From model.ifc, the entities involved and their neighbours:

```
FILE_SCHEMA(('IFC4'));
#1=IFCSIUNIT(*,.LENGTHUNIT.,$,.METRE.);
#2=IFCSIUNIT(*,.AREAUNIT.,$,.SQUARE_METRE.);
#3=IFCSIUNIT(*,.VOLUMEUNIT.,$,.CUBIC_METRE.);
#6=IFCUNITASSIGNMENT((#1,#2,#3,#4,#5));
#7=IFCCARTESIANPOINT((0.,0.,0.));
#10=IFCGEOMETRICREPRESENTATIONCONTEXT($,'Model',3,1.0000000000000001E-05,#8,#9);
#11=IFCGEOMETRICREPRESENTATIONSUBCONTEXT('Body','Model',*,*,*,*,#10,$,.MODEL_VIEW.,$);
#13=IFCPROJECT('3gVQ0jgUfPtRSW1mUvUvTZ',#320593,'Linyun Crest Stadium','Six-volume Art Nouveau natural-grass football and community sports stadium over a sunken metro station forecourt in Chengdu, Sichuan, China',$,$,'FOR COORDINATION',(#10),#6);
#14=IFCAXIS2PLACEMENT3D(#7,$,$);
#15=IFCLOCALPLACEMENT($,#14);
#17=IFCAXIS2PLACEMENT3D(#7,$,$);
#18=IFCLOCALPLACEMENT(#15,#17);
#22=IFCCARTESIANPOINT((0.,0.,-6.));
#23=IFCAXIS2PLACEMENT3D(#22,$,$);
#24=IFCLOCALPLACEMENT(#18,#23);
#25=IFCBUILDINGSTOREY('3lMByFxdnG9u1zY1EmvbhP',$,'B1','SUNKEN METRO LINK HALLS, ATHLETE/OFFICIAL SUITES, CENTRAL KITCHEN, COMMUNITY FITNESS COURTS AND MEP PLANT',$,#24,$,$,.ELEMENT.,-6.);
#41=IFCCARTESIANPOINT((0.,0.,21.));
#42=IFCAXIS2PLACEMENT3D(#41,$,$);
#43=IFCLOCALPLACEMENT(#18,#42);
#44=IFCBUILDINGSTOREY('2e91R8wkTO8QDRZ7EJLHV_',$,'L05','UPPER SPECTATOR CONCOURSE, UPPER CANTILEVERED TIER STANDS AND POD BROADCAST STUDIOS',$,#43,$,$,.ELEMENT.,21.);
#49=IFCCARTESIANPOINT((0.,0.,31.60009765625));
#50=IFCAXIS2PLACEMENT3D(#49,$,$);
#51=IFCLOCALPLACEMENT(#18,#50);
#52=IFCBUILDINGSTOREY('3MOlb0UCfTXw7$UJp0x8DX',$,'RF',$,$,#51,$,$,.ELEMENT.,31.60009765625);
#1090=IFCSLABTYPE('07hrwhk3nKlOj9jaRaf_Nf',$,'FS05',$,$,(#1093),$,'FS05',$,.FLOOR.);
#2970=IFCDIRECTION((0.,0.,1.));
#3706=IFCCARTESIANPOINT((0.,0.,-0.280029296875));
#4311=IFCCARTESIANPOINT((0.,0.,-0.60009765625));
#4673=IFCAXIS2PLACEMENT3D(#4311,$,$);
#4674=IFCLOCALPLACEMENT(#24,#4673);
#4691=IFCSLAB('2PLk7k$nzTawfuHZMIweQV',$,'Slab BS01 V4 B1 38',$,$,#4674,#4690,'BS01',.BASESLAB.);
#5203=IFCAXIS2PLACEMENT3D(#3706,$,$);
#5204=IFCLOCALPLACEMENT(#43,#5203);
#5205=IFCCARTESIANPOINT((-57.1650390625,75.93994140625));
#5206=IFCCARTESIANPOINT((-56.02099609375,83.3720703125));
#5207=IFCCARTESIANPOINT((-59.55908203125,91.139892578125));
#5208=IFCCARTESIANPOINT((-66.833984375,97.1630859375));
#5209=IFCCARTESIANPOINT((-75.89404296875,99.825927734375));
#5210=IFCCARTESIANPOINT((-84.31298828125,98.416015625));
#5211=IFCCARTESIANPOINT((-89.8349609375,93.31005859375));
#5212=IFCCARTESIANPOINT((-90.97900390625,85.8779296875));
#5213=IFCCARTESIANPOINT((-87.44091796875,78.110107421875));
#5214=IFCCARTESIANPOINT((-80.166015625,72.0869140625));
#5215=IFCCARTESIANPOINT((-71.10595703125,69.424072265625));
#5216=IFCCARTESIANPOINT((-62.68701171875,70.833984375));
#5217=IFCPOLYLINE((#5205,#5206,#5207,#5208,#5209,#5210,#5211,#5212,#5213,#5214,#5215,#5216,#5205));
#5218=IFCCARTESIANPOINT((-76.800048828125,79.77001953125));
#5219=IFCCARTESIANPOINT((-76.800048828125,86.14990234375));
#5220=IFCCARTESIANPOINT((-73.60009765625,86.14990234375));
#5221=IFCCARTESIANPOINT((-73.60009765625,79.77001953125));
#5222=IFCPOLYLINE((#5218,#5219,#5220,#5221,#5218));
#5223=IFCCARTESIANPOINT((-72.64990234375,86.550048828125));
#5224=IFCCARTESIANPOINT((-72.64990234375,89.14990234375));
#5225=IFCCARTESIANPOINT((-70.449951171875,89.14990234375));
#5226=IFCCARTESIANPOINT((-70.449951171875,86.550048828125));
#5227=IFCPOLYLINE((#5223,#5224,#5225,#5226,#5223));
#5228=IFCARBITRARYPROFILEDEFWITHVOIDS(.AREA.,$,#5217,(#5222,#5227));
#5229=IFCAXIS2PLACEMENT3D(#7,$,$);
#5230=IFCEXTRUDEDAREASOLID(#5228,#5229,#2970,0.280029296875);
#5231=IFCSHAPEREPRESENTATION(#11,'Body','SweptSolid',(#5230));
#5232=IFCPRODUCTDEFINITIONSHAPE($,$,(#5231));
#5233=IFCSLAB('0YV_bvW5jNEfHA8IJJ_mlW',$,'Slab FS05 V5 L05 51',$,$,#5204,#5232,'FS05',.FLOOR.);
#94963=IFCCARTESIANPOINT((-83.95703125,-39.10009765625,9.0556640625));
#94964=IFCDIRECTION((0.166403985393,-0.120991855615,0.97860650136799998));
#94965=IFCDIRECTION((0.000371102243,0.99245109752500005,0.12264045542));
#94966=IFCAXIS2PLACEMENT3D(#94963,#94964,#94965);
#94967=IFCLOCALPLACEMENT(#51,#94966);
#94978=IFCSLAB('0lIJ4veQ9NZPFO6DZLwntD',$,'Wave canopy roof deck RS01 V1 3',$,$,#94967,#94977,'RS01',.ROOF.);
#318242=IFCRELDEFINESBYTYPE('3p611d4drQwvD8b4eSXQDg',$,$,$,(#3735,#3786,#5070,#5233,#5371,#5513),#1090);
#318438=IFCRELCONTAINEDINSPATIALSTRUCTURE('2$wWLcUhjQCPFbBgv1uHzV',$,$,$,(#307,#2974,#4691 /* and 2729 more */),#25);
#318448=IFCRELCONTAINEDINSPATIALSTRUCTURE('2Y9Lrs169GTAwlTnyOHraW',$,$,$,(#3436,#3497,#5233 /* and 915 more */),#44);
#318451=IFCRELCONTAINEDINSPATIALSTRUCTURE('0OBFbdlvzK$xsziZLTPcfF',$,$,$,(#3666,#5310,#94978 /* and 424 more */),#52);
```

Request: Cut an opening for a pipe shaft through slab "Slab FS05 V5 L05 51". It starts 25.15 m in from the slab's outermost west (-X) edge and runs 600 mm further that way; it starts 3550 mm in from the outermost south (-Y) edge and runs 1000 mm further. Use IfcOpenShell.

```python
import numpy as np
import ifcopenshell
import ifcopenshell.api.feature
import ifcopenshell.api.geometry
import ifcopenshell.api.root
import ifcopenshell.geom
import ifcopenshell.util.placement
import ifcopenshell.util.representation
import ifcopenshell.util.shape
import ifcopenshell.util.unit

model = ifcopenshell.open("model.ifc")
unit_scale = ifcopenshell.util.unit.calculate_unit_scale(model)
settings = ifcopenshell.geom.settings()


def volume(element):
    """Net volume in cubic metres, openings subtracted."""
    shape = ifcopenshell.geom.create_shape(settings, element)
    return ifcopenshell.util.shape.get_volume(shape.geometry)


slab = model.by_id(5233)
before = volume(slab)

# Extent in the slab's own axes, in metres. The edges named are its -X and -Y sides.
slab_shape = ifcopenshell.geom.create_shape(settings, slab)
vertices = ifcopenshell.util.shape.get_vertices(slab_shape.geometry)
x_min, y_min, bottom = vertices.min(axis=0)
top = vertices[:, 2].max()

opening = ifcopenshell.api.root.create_entity(model, ifc_class="IfcOpeningElement", name="Pipe shaft opening", predefined_type="OPENING")
context = ifcopenshell.util.representation.get_context(model, "Model", "Body", "MODEL_VIEW")
width, depth = 0.6, 1
outline = [(0.0, 0.0), (width, 0.0), (width, depth), (0.0, depth), (0.0, 0.0)]
# Overshoot both faces by 50 mm so the cut is clean.
shape = ifcopenshell.api.geometry.add_slab_representation(
    model, context=context, depth=top - bottom + 0.1, polyline=outline
)
ifcopenshell.api.geometry.assign_representation(model, product=opening, representation=shape)

matrix = ifcopenshell.util.placement.get_local_placement(slab.ObjectPlacement)
matrix[:, 3] = matrix @ np.append(np.array([x_min + 25.15, y_min + 3.55, bottom - 0.05]) / unit_scale, 1.0)
ifcopenshell.api.geometry.edit_object_placement(model, product=opening, matrix=matrix, is_si=False)
ifcopenshell.api.feature.add_feature(model, feature=opening, element=slab)

after = volume(slab)

print(f"slab volume {before:.3f} -> {after:.3f} m3")

model.write("model-out.ifc")
```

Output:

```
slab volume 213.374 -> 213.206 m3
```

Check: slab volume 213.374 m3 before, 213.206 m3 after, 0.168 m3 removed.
